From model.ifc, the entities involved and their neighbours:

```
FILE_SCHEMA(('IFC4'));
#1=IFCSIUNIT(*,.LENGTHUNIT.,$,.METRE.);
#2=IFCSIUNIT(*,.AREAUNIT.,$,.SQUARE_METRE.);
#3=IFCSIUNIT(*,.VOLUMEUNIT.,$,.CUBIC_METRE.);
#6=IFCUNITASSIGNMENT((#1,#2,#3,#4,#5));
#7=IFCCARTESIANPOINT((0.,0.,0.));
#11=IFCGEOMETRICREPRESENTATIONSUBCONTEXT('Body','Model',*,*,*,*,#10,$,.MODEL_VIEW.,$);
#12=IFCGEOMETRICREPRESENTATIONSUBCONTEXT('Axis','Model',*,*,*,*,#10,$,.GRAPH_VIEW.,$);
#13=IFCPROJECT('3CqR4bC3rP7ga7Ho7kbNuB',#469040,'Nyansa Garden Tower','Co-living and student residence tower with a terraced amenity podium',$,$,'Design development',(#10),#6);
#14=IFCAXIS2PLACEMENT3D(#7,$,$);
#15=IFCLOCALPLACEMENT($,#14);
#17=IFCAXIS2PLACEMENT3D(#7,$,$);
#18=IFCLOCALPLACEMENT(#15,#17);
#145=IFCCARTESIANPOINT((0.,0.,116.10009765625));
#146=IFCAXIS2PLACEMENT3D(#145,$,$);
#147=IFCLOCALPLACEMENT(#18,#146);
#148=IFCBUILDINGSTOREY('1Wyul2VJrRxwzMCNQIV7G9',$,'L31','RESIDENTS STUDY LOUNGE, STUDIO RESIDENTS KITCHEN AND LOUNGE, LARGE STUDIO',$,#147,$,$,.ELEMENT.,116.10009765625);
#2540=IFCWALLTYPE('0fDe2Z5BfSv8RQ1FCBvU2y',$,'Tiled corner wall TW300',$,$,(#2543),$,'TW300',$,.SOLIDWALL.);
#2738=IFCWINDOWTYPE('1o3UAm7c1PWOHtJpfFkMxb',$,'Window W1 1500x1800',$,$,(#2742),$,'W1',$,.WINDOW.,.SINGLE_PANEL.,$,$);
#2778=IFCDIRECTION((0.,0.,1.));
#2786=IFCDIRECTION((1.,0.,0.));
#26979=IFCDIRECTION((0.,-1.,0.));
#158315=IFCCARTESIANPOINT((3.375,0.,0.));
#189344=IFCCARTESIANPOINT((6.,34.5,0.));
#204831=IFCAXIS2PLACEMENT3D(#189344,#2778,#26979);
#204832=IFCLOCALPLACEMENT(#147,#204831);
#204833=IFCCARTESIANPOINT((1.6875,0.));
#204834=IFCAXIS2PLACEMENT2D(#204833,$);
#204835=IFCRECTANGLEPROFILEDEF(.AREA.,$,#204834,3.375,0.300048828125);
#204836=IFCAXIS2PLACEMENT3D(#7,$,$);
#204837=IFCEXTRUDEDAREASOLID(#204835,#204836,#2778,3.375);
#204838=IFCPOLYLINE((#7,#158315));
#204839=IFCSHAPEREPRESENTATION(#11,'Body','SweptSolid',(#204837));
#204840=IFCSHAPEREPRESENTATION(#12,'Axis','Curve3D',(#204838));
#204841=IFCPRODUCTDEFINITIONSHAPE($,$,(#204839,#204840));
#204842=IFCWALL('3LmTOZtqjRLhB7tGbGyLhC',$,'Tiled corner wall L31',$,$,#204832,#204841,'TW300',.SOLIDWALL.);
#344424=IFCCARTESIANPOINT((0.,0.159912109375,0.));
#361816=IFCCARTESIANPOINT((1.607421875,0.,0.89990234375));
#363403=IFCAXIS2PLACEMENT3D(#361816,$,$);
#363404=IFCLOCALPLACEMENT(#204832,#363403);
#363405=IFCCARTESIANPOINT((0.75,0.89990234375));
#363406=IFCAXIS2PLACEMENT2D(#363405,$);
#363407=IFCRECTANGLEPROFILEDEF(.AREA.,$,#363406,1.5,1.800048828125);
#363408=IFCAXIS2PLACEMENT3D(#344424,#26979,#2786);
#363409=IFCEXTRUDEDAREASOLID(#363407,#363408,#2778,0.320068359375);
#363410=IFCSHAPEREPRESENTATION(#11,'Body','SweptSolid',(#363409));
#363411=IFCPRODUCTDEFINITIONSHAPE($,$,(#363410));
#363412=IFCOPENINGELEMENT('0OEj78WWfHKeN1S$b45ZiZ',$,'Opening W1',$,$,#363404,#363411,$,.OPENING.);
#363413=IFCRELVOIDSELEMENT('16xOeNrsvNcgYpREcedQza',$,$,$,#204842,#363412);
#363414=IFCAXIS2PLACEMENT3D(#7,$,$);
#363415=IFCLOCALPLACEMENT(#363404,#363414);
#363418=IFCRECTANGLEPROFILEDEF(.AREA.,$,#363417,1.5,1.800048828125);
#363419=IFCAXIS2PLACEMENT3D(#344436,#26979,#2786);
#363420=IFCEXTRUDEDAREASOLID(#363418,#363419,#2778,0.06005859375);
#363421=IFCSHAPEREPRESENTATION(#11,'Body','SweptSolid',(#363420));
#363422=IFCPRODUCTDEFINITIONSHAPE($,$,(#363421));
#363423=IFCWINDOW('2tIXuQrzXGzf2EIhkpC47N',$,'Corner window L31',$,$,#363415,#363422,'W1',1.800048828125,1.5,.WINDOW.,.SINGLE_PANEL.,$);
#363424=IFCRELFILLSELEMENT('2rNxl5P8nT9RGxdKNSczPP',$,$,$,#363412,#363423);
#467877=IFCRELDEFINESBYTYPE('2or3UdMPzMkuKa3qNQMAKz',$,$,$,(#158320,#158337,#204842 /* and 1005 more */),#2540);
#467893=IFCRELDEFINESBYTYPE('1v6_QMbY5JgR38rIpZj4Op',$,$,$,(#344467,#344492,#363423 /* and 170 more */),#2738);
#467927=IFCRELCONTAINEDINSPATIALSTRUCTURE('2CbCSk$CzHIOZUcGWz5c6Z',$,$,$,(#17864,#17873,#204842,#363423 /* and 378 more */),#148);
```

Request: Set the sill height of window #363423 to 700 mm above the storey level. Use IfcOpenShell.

```python
import numpy as np
import ifcopenshell
import ifcopenshell.api.geometry
import ifcopenshell.geom
import ifcopenshell.util.element
import ifcopenshell.util.placement
import ifcopenshell.util.shape
import ifcopenshell.util.unit

model = ifcopenshell.open("model.ifc")
unit_scale = ifcopenshell.util.unit.calculate_unit_scale(model)

window = model.by_guid("2tIXuQrzXGzf2EIhkpC47N")
opening = window.FillsVoids[0].RelatingOpeningElement
storey = ifcopenshell.util.element.get_container(window, ifc_class="IfcBuildingStorey")
level = ifcopenshell.util.placement.get_local_placement(storey.ObjectPlacement)[2, 3]

# The opening's origin need not be at the sill, so measure its lowest point.
shape = ifcopenshell.geom.create_shape(ifcopenshell.geom.settings(), opening)
bottom = ifcopenshell.util.shape.get_shape_bottom_elevation(shape, shape.geometry) / unit_scale
dz = level + 0.7 / unit_scale - bottom

shift = np.array([0.0, 0.0, dz])
# The window is placed relative to its opening, so it follows when the opening moves.
matrix = ifcopenshell.util.placement.get_local_placement(opening.ObjectPlacement)
matrix[:3, 3] += shift
ifcopenshell.api.geometry.edit_object_placement(
    model, product=opening, matrix=matrix, is_si=False, should_transform_children=True
)

print(f"moved by {dz * unit_scale:+.3f} m")

model.write("model_edited.ifc")
```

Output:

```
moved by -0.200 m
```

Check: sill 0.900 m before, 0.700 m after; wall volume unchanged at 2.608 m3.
